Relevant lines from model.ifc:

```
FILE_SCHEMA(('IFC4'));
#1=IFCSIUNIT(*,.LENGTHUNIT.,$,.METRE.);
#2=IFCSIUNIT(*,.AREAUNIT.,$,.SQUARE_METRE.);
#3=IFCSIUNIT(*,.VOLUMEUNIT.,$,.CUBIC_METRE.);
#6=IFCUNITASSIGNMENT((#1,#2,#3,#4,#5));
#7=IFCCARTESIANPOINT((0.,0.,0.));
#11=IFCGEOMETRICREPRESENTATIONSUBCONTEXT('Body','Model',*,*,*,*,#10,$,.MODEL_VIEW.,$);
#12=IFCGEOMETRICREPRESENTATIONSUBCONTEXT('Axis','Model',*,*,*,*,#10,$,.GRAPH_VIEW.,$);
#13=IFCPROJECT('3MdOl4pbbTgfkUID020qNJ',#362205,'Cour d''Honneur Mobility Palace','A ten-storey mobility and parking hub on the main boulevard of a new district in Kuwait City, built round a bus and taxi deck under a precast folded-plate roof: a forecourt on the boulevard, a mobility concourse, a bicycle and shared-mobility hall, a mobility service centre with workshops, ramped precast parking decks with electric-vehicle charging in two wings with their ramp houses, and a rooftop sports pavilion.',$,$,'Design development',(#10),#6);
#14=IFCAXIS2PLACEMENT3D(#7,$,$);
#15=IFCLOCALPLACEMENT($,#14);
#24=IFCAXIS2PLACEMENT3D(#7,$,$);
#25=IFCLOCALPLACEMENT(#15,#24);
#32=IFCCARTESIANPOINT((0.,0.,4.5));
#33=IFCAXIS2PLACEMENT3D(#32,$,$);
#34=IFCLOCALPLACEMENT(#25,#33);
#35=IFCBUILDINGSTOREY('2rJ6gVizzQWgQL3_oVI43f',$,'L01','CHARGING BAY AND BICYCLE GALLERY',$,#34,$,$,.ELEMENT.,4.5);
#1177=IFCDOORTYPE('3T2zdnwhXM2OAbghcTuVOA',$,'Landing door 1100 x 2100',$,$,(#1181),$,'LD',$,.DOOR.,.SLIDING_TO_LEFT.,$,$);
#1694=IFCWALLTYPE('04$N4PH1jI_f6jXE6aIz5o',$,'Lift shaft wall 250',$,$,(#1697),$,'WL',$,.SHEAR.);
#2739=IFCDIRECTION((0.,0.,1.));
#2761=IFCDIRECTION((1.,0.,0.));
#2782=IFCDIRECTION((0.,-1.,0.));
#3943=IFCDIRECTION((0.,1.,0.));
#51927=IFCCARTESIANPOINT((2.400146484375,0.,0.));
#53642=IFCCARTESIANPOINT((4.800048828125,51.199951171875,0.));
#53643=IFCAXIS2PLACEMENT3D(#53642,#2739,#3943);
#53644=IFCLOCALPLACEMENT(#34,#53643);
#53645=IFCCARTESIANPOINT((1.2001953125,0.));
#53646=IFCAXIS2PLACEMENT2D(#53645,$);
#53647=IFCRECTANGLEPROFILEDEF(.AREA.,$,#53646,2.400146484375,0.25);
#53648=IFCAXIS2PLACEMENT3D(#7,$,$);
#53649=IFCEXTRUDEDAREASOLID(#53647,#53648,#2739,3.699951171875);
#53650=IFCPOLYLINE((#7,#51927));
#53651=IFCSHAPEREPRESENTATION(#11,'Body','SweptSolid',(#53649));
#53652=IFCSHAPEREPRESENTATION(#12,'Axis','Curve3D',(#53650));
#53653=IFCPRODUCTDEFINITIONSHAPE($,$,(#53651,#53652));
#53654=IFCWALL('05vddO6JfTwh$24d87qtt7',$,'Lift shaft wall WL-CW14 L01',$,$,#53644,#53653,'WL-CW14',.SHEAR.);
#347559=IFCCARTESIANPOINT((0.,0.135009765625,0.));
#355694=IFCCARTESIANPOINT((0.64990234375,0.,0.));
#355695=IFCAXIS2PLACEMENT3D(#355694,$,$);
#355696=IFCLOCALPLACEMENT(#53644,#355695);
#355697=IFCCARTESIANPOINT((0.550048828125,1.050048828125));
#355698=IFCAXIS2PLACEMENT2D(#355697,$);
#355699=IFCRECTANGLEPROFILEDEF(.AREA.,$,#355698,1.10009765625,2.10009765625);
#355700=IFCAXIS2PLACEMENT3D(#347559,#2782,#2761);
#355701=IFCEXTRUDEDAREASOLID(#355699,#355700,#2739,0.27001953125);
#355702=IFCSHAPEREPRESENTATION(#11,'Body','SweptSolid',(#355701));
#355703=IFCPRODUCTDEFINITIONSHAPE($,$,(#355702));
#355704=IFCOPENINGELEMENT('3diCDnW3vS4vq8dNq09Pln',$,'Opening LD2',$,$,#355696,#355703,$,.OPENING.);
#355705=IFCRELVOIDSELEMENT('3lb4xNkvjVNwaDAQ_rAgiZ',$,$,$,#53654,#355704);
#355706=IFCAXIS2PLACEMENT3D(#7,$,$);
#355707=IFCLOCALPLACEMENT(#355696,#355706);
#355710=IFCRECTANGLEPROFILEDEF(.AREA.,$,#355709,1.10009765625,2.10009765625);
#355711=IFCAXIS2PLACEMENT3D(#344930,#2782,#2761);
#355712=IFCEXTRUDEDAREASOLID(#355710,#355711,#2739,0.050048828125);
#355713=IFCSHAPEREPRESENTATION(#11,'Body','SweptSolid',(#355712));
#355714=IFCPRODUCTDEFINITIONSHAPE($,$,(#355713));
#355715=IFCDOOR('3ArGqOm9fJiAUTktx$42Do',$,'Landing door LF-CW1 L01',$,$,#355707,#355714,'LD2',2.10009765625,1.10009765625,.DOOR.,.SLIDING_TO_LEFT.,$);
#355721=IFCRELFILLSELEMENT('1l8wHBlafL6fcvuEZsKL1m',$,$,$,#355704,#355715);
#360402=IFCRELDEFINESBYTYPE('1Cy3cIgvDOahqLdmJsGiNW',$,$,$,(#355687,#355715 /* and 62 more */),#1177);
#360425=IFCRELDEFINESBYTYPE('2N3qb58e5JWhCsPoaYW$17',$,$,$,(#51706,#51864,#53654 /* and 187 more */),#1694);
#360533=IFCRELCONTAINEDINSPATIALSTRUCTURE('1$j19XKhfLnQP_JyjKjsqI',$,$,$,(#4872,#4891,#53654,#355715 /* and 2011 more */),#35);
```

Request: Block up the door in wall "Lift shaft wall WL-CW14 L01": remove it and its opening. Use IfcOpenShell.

```python
import ifcopenshell
import ifcopenshell.api.feature
import ifcopenshell.api.root
import ifcopenshell.geom
import ifcopenshell.util.shape

model = ifcopenshell.open("model.ifc")
settings = ifcopenshell.geom.settings()


def volume(element):
    """Net volume in cubic metres, openings subtracted."""
    shape = ifcopenshell.geom.create_shape(settings, element)
    return ifcopenshell.util.shape.get_volume(shape.geometry)


door = model.by_guid("3ArGqOm9fJiAUTktx$42Do")
opening = door.FillsVoids[0].RelatingOpeningElement
wall = opening.VoidsElements[0].RelatingBuildingElement
before = volume(wall)

ifcopenshell.api.root.remove_product(model, product=door)
ifcopenshell.api.feature.remove_feature(model, feature=opening)

after = volume(wall)

print(f"wall volume {before:.3f} -> {after:.3f} m3")

model.write("model_rev.ifc")
```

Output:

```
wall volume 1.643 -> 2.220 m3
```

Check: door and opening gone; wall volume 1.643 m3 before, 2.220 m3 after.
